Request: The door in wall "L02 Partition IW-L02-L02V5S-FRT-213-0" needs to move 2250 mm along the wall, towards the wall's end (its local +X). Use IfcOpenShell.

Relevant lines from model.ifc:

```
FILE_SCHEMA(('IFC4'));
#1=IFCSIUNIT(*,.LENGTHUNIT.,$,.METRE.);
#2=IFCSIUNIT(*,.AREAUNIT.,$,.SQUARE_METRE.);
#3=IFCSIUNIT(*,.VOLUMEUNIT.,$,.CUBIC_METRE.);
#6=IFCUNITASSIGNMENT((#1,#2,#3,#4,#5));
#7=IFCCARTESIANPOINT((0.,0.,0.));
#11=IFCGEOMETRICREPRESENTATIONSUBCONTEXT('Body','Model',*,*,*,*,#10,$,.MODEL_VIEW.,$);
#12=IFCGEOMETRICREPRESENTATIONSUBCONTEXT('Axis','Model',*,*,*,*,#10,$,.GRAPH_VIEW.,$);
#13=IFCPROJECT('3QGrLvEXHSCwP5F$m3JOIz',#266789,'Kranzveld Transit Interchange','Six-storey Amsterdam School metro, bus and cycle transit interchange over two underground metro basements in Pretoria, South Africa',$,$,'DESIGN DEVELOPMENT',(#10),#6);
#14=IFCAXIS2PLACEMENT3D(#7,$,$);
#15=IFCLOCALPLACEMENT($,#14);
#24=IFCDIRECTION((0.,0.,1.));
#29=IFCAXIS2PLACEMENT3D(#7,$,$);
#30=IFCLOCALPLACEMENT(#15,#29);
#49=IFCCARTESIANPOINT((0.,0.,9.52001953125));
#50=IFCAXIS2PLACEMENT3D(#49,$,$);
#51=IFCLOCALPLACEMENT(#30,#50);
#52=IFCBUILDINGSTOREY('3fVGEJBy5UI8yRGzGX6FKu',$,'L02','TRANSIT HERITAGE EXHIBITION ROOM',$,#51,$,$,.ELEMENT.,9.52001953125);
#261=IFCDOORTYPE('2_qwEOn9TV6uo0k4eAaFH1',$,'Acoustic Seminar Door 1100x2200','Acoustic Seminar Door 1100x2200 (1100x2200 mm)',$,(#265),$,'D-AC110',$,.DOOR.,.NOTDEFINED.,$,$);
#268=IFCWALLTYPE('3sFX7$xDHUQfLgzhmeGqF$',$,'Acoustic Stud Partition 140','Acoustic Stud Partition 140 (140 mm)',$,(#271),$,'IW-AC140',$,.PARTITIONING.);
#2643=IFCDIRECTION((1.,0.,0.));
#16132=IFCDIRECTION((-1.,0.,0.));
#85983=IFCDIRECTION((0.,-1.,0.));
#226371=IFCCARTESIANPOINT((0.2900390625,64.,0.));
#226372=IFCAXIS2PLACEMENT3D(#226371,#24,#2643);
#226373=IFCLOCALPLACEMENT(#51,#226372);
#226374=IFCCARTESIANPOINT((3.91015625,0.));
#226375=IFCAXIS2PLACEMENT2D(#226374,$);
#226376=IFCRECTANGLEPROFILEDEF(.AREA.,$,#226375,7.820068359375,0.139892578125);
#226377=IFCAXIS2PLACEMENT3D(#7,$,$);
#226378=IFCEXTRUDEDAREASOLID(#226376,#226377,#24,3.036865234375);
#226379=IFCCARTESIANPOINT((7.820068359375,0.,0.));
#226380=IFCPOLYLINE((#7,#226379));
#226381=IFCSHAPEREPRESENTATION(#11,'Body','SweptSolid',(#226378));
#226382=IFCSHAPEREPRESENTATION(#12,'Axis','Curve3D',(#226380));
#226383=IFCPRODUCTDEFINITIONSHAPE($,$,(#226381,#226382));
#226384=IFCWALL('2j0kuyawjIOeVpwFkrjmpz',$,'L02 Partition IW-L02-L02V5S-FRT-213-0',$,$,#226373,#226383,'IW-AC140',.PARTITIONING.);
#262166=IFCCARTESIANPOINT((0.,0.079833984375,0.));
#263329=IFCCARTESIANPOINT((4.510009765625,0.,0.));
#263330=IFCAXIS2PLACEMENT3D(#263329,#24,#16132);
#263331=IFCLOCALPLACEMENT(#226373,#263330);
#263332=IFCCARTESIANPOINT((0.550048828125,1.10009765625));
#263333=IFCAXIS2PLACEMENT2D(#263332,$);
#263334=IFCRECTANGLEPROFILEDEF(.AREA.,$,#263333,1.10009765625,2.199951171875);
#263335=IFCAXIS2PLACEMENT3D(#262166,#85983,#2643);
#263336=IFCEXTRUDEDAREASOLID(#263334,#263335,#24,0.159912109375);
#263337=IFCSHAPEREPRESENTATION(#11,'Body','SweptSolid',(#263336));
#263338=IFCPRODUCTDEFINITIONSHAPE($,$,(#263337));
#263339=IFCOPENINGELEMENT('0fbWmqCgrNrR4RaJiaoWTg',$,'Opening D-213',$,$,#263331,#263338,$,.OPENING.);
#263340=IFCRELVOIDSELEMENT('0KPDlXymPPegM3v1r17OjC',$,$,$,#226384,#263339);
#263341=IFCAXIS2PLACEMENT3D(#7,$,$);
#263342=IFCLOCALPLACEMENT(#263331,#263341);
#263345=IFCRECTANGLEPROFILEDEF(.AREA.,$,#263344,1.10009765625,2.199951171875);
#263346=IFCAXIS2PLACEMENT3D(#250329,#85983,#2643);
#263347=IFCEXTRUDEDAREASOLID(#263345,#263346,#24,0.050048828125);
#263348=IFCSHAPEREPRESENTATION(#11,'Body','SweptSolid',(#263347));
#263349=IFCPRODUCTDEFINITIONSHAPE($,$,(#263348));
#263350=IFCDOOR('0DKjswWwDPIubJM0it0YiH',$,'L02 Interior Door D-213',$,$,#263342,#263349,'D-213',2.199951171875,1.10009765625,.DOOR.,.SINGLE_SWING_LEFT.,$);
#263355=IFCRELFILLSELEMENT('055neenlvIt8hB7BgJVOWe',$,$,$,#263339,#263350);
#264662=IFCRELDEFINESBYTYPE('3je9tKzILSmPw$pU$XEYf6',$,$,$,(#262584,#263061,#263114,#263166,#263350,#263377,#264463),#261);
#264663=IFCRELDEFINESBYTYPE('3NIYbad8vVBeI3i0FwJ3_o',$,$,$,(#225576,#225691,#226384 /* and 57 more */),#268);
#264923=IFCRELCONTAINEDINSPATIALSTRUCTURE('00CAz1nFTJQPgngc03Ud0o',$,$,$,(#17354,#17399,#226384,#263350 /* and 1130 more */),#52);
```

```python
import ifcopenshell
import ifcopenshell.api.geometry
import ifcopenshell.util.placement

model = ifcopenshell.open("model.ifc")

door = model.by_id(263350)
opening = door.FillsVoids[0].RelatingOpeningElement
wall = opening.VoidsElements[0].RelatingBuildingElement

wall_matrix = ifcopenshell.util.placement.get_local_placement(wall.ObjectPlacement)
shift = wall_matrix[:3, 0] * 2.25
before = ifcopenshell.util.placement.get_local_placement(door.ObjectPlacement)[:3, 3].copy()

# The door is placed relative to its opening, so it follows when the opening moves.
matrix = ifcopenshell.util.placement.get_local_placement(opening.ObjectPlacement)
matrix[:3, 3] += shift
ifcopenshell.api.geometry.edit_object_placement(
    model, product=opening, matrix=matrix, is_si=False, should_transform_children=True
)

after = ifcopenshell.util.placement.get_local_placement(door.ObjectPlacement)[:3, 3]
print("door moved by", (after - before).round(3) + 0.0)

model.write("model_v2.ifc")
```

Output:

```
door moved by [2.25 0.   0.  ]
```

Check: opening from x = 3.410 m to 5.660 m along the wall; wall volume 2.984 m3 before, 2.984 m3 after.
